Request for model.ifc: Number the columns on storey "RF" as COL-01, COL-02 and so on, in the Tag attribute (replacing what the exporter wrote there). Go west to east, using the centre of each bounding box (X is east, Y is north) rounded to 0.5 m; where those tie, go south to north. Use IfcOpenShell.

First a look at what the model holds.

```python
import ifcopenshell
import ifcopenshell.util.element
import ifcopenshell.util.placement

model = ifcopenshell.open("model.ifc")
print(model.schema)
storey = next(s for s in model.by_type("IfcBuildingStorey") if s.Name == "RF")
columns = [e for e in ifcopenshell.util.element.get_decomposition(storey) if e.is_a("IfcColumn")]
for e in sorted(columns, key=lambda e: e.id()):
    origin = ifcopenshell.util.placement.get_local_placement(e.ObjectPlacement)[:3, 3]
    print(e.id(), e.Tag, e.Name, origin.round(2) + 0.0, sep=" | ")
```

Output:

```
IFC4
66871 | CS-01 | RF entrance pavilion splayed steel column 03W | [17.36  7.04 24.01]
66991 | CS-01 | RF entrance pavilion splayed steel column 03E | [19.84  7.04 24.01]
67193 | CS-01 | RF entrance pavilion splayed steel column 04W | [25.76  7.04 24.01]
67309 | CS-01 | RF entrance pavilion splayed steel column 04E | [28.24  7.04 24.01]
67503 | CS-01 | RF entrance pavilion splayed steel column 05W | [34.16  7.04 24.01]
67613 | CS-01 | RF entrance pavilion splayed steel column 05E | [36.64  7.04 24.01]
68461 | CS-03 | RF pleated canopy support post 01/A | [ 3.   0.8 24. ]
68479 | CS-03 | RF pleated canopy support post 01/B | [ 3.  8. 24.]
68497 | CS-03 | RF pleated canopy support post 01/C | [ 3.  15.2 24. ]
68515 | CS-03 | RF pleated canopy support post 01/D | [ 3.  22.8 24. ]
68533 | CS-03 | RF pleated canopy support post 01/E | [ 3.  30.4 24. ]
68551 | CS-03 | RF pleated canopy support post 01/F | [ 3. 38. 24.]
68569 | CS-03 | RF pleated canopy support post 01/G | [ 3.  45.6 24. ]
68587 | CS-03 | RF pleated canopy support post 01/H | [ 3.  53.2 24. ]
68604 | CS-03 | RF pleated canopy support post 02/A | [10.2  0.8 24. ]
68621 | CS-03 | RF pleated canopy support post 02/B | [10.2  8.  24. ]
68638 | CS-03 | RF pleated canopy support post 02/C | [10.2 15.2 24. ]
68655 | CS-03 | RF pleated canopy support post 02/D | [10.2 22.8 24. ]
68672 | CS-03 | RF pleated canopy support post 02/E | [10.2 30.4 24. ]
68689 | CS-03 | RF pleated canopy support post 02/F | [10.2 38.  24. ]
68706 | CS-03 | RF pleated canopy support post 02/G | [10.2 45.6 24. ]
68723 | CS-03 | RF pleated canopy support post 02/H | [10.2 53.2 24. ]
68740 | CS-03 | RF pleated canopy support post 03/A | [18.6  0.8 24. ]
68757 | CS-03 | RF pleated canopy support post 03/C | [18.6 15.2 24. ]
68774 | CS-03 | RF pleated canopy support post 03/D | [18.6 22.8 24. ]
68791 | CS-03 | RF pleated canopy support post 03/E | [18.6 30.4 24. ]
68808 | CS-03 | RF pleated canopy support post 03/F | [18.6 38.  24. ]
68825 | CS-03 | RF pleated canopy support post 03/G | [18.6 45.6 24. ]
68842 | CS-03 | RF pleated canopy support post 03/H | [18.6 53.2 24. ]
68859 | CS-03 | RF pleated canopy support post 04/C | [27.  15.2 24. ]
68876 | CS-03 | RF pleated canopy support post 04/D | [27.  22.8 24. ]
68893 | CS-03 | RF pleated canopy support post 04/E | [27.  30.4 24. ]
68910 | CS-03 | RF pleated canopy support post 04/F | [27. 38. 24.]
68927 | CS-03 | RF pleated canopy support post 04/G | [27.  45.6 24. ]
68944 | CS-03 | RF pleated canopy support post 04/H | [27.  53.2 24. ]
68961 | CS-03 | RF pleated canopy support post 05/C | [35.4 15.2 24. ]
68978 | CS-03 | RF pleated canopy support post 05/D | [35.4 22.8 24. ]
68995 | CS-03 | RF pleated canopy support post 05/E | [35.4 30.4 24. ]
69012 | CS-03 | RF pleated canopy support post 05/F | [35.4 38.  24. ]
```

```python
import ifcopenshell
import ifcopenshell.geom
import ifcopenshell.util.element
import ifcopenshell.util.shape

model = ifcopenshell.open("model.ifc")
settings = ifcopenshell.geom.settings()
settings.set("use-world-coords", True)


def centre(element):
    shape = ifcopenshell.geom.create_shape(settings, element)
    return ifcopenshell.util.shape.get_bbox_centroid(shape.geometry)


storey = next(s for s in model.by_type("IfcBuildingStorey") if s.Name == "RF")
columns = [e for e in ifcopenshell.util.element.get_decomposition(storey) if e.is_a("IfcColumn")]

# Insertion points can sit at a corner or the storey origin, so sort by the geometry (in metres).
centres = {e: centre(e) for e in columns}
columns.sort(key=lambda e: (round(centres[e][0] / 0.5), centres[e][1]))

for i, e in enumerate(columns, start=1):
    number = f"COL-{i:02d}"
    e.Tag = number
    print(e.id(), number)

model.write("model_updated.ifc")
```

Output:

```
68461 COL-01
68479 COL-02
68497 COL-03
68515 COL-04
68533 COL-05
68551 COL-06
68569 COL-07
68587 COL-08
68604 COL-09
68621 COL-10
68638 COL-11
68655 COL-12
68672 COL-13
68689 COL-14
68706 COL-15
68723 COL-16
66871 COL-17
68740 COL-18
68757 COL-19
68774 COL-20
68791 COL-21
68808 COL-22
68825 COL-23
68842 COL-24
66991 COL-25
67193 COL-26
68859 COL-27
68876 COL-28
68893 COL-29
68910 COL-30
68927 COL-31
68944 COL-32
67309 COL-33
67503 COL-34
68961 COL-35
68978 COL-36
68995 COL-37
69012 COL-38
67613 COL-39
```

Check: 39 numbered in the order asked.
